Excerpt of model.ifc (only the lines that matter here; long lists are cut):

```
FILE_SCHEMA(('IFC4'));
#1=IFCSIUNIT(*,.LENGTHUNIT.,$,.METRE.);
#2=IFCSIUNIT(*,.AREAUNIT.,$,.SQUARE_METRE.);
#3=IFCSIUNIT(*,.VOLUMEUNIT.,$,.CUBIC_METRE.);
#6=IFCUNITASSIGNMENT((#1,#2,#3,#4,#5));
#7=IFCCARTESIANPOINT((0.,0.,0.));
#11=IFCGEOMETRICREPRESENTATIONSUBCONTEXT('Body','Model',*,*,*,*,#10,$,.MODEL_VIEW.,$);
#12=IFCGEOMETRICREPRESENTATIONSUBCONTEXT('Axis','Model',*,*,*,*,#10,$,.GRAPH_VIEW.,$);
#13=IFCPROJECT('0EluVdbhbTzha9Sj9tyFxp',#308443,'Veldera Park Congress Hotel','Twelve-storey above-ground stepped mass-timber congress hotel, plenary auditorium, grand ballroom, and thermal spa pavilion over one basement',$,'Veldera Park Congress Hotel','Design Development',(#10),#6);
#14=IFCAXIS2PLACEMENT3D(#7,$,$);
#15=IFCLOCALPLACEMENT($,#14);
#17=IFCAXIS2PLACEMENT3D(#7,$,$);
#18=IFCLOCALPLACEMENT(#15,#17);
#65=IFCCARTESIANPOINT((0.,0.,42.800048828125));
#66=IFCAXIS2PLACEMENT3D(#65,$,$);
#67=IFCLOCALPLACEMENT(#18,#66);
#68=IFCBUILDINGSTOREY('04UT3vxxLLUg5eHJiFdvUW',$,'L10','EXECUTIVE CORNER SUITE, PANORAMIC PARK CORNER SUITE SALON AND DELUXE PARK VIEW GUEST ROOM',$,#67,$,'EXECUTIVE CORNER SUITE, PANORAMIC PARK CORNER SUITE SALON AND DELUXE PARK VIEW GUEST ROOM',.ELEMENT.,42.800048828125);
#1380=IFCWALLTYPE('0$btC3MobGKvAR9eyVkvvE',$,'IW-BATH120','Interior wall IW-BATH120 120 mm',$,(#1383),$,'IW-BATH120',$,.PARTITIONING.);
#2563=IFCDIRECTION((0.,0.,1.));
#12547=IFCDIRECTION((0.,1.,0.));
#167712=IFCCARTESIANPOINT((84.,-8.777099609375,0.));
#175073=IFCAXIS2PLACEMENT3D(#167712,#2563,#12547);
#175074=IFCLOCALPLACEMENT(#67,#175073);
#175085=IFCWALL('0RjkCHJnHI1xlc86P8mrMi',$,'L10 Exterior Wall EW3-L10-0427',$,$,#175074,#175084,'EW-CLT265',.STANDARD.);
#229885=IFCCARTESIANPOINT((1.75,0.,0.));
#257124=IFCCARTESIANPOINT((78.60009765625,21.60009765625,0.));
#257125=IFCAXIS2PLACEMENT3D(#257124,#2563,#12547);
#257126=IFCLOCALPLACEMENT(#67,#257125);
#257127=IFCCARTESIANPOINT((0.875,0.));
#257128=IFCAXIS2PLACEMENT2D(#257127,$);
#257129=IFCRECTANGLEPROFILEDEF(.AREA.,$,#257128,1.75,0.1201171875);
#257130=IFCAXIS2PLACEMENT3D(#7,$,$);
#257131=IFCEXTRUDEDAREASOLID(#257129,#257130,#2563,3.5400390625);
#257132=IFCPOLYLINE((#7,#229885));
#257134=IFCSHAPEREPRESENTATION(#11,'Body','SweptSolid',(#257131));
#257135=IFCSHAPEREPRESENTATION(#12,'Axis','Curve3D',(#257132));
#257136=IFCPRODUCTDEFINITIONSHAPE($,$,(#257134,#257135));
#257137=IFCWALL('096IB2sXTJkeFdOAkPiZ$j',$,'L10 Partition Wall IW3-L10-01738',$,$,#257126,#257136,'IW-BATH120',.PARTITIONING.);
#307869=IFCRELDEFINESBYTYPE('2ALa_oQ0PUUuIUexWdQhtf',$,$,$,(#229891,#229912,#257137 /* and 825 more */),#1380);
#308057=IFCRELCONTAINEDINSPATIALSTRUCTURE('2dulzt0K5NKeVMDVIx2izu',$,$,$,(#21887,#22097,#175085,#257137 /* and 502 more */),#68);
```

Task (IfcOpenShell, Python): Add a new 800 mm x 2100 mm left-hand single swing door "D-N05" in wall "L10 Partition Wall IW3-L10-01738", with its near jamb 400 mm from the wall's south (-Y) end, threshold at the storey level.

```python
import numpy as np
import ifcopenshell
import ifcopenshell.api.feature
import ifcopenshell.api.geometry
import ifcopenshell.api.root
import ifcopenshell.api.spatial
import ifcopenshell.geom
import ifcopenshell.util.element
import ifcopenshell.util.placement
import ifcopenshell.util.representation
import ifcopenshell.util.shape
import ifcopenshell.util.unit

model = ifcopenshell.open("model.ifc")
unit_scale = ifcopenshell.util.unit.calculate_unit_scale(model)
settings = ifcopenshell.geom.settings()


def volume(element):
    """Net volume in cubic metres, openings subtracted."""
    shape = ifcopenshell.geom.create_shape(settings, element)
    return ifcopenshell.util.shape.get_volume(shape.geometry)


wall = model.by_id(257137)
storey = ifcopenshell.util.element.get_container(wall, ifc_class="IfcBuildingStorey")
context = ifcopenshell.util.representation.get_context(model, "Model", "Body", "MODEL_VIEW")
before = volume(wall)

width, height, from_end, sill = 0.8, 2.1, 0.4, 0.0  # metres

# The wall runs along its own X axis, and the end named is its -X end.
wall_shape = ifcopenshell.geom.create_shape(settings, wall)
x, y, z = ifcopenshell.util.shape.get_vertices(wall_shape.geometry).T
start = x.min() + from_end
face, thickness = float(y.min()), float(y.max() - y.min())
wall_matrix = ifcopenshell.util.placement.get_local_placement(wall.ObjectPlacement)
level = ifcopenshell.util.placement.get_local_placement(storey.ObjectPlacement)[2, 3]


def in_wall(x, y):
    """Placement at x, y metres in the wall's axes, at sill height."""
    matrix = wall_matrix.copy()
    matrix[:, 3] = wall_matrix @ np.array([x / unit_scale, y / unit_scale, 0.0, 1.0])
    matrix[2, 3] = level + sill / unit_scale
    return matrix


# Opening: a box that overshoots both wall faces by 50 mm.
opening = ifcopenshell.api.root.create_entity(model, ifc_class="IfcOpeningElement", predefined_type="OPENING")
box = ifcopenshell.api.geometry.add_wall_representation(
    model, context=context, length=width, height=height, thickness=thickness + 0.1
)
ifcopenshell.api.geometry.assign_representation(model, product=opening, representation=box)
ifcopenshell.api.geometry.edit_object_placement(model, product=opening, matrix=in_wall(start, face - 0.05), is_si=False)
ifcopenshell.api.feature.add_feature(model, feature=opening, element=wall)

door = ifcopenshell.api.root.create_entity(model, ifc_class="IfcDoor", name="D-N05", predefined_type="DOOR")
door.OverallWidth, door.OverallHeight = width / unit_scale, height / unit_scale
door.OperationType = "SINGLE_SWING_LEFT"
body = ifcopenshell.api.geometry.add_door_representation(
    model,
    context=context,
    overall_width=door.OverallWidth,
    overall_height=door.OverallHeight,
    operation_type="SINGLE_SWING_LEFT",
    lining_properties={"LiningDepth": thickness / unit_scale, "ThresholdDepth": thickness / unit_scale},
)
ifcopenshell.api.geometry.assign_representation(model, product=door, representation=body)
ifcopenshell.api.spatial.assign_container(model, products=[door], relating_structure=storey)
ifcopenshell.api.feature.add_filling(model, opening=opening, element=door)

# The lining spans the wall, so the door starts at the wall face.
ifcopenshell.api.geometry.edit_object_placement(model, product=door, matrix=in_wall(start, face), is_si=False)

after = volume(wall)

print(f"wall volume {before:.3f} -> {after:.3f} m3")

model.write("model-out.ifc")
```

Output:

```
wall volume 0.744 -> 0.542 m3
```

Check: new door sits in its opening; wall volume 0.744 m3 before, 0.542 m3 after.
